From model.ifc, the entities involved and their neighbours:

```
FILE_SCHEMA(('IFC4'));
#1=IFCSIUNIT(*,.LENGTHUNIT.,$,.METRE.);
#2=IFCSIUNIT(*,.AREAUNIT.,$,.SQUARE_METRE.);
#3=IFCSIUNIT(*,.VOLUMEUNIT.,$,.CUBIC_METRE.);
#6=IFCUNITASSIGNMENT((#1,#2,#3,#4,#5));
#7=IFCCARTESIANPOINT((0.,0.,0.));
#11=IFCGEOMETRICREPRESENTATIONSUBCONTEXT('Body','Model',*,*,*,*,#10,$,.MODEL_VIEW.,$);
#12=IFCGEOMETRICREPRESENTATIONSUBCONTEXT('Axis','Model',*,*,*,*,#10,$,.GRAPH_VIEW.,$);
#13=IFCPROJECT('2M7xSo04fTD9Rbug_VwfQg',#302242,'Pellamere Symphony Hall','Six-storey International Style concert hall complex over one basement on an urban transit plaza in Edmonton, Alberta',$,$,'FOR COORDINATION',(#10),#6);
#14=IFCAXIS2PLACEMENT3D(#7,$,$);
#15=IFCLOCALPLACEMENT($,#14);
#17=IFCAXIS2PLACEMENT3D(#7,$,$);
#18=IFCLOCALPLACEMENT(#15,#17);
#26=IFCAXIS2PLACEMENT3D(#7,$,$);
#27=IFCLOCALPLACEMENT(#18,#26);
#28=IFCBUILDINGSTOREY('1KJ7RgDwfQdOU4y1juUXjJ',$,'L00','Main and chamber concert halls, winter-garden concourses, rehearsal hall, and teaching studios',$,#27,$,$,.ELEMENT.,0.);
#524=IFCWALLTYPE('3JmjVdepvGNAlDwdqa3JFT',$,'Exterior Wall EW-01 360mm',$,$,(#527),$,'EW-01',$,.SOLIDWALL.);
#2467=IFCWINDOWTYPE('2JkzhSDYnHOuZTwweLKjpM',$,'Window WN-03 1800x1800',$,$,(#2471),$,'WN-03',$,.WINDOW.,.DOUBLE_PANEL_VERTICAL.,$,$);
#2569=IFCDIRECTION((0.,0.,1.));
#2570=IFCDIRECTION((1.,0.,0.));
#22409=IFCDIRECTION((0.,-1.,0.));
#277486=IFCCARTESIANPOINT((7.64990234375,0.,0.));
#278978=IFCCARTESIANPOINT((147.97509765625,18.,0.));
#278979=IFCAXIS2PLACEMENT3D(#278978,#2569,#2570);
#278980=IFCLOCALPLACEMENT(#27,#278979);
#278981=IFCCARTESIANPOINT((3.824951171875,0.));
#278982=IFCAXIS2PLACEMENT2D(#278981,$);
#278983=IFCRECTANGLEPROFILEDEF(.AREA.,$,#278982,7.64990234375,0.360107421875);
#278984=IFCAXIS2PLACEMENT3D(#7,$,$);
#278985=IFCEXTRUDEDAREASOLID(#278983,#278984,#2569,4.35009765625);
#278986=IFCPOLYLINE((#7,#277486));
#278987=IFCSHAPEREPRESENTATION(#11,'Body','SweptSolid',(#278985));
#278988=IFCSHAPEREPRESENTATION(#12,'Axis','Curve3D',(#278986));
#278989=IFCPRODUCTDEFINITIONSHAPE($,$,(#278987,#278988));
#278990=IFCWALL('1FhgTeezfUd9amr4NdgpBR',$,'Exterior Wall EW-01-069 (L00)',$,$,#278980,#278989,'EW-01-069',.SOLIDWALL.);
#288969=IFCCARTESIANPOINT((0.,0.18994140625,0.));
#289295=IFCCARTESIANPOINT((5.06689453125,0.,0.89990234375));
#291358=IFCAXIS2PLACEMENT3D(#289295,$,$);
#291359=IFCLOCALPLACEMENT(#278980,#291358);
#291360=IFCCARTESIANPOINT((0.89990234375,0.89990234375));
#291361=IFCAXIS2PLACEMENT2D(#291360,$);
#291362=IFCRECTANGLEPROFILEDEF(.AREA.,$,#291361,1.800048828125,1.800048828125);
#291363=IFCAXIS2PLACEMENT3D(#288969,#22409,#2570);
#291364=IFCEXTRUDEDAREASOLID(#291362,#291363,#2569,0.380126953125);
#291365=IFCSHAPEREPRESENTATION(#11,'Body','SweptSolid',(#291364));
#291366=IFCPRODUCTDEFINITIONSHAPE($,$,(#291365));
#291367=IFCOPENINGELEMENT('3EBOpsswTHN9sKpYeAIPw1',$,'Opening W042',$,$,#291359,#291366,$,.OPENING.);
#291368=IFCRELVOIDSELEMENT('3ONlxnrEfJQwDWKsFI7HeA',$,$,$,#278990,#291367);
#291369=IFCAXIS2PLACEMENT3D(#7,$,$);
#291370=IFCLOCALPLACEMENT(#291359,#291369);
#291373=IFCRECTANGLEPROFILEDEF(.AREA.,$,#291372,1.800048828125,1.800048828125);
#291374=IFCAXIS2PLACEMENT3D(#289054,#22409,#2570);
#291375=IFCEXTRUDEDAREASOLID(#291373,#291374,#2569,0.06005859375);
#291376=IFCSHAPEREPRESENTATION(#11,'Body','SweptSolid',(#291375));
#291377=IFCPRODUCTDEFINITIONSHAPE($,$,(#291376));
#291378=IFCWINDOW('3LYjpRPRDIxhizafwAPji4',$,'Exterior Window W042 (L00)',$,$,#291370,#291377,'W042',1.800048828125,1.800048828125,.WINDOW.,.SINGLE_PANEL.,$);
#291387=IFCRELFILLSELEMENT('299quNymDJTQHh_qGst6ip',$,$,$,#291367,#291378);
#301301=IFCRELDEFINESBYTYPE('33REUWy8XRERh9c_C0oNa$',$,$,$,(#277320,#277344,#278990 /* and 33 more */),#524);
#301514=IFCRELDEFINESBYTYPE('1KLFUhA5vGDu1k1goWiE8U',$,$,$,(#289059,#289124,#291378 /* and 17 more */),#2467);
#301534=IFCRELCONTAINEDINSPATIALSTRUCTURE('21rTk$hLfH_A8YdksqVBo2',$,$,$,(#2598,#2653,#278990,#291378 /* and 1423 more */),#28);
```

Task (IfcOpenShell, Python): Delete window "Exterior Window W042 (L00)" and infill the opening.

```python
import ifcopenshell
import ifcopenshell.api.feature
import ifcopenshell.api.root
import ifcopenshell.geom
import ifcopenshell.util.shape

model = ifcopenshell.open("model.ifc")
settings = ifcopenshell.geom.settings()


def volume(element):
    """Net volume in cubic metres, openings subtracted."""
    shape = ifcopenshell.geom.create_shape(settings, element)
    return ifcopenshell.util.shape.get_volume(shape.geometry)


window = model.by_id(291378)
opening = window.FillsVoids[0].RelatingOpeningElement
wall = opening.VoidsElements[0].RelatingBuildingElement
before = volume(wall)

ifcopenshell.api.root.remove_product(model, product=window)
ifcopenshell.api.feature.remove_feature(model, feature=opening)

after = volume(wall)

print(f"wall volume {before:.3f} -> {after:.3f} m3")

model.write("model-out.ifc")
```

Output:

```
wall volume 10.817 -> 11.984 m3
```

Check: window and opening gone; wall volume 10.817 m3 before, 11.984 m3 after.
